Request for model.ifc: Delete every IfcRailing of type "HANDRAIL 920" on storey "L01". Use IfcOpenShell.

First a look at what the model holds.

```python
import ifcopenshell
import ifcopenshell.util.element

model = ifcopenshell.open("model.ifc")
print(model.schema)
storey = next(s for s in model.by_type("IfcBuildingStorey") if s.Name == "L01")
railings = [e for e in ifcopenshell.util.element.get_decomposition(storey) if e.is_a("IfcRailing")]
seen = {}
for e in railings:
    element_type = ifcopenshell.util.element.get_type(e)
    name = element_type.Name if element_type not in (None, e) else None
    seen[name] = seen.get(name, 0) + 1
for name, count in sorted(seen.items(), key=str):
    print(count, "x", name)
```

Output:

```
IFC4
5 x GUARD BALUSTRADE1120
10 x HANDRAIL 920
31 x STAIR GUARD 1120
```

```python
import ifcopenshell
import ifcopenshell.api.root
import ifcopenshell.util.element

model = ifcopenshell.open("model.ifc")

storey = next(s for s in model.by_type("IfcBuildingStorey") if s.Name == "L01")
railings = [e for e in ifcopenshell.util.element.get_decomposition(storey) if e.is_a("IfcRailing")]
targets = [e for e in railings if (t := ifcopenshell.util.element.get_type(e)) not in (None, e) and t.Name == "HANDRAIL 920"]

for e in targets:
    ifcopenshell.api.root.remove_product(model, product=e)
print(len(targets), "removed")

model.write("model_edited.ifc")
```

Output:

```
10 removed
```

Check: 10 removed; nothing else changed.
